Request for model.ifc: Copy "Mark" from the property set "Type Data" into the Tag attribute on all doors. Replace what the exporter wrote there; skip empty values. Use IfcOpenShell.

First a look at what the model holds.

```python
import ifcopenshell
import ifcopenshell.util.element

model = ifcopenshell.open("model.ifc")
print(model.schema)
doors = model.by_type("IfcDoor")
print(len(doors), "doors")
for e in doors[:8]:
    source = ifcopenshell.util.element.get_pset(e, "Type Data", "Mark")
    target = e.Tag
    print(e.id(), repr(source), repr(target), sep=" | ")
```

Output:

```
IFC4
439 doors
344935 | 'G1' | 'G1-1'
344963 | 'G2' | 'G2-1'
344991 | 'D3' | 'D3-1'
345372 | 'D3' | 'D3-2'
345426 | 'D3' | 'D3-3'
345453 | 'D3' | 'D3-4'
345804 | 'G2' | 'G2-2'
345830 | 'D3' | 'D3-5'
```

```python
import ifcopenshell
import ifcopenshell.util.element

model = ifcopenshell.open("model.ifc")

count = 0
for e in model.by_type("IfcDoor"):
    value = ifcopenshell.util.element.get_pset(e, "Type Data", "Mark")
    current = e.Tag
    if not value or not value.strip() or current == value:
        continue
    e.Tag = value
    count += 1

print(count, "doors updated")

model.write("model_updated.ifc")
```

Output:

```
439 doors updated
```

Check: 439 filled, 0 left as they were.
